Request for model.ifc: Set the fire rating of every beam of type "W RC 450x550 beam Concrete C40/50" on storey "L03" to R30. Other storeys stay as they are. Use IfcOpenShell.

First a look at what the model holds.

```python
import ifcopenshell
import ifcopenshell.util.element

model = ifcopenshell.open("model.ifc")
print(model.schema)
storey = next(s for s in model.by_type("IfcBuildingStorey") if s.Name == "L03")
beams = [e for e in ifcopenshell.util.element.get_decomposition(storey) if e.is_a("IfcBeam")]
seen = {}
for e in beams:
    element_type = ifcopenshell.util.element.get_type(e)
    key = (element_type.Name if element_type != e and element_type else None, ifcopenshell.util.element.get_pset(e, "Pset_BeamCommon", "FireRating"))
    seen[key] = seen.get(key, 0) + 1
for (name, value), count in sorted(seen.items(), key=str):
    print(count, "x", name, "|", value)
```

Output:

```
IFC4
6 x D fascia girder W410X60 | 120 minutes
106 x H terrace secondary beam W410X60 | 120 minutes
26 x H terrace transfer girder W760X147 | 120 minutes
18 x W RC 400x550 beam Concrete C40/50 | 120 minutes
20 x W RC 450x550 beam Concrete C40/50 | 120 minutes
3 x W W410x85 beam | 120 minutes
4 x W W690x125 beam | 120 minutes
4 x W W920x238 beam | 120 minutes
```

```python
import ifcopenshell
import ifcopenshell.api.pset
import ifcopenshell.util.element

model = ifcopenshell.open("model.ifc")

storey = next(s for s in model.by_type("IfcBuildingStorey") if s.Name == "L03")
beams = [e for e in ifcopenshell.util.element.get_decomposition(storey) if e.is_a("IfcBeam")]

count = 0
for e in beams:
    element_type = ifcopenshell.util.element.get_type(e)
    if element_type in (None, e) or element_type.Name != "W RC 450x550 beam Concrete C40/50":
        continue
    # add_pset returns the element's existing set when there is one.
    pset = ifcopenshell.api.pset.add_pset(model, product=e, name="Pset_BeamCommon")
    ifcopenshell.api.pset.edit_pset(model, pset=pset, properties={"FireRating": "R30"})
    count += 1

print(count, "beams updated")

model.write("model_updated.ifc")
```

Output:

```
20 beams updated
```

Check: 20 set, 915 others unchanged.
